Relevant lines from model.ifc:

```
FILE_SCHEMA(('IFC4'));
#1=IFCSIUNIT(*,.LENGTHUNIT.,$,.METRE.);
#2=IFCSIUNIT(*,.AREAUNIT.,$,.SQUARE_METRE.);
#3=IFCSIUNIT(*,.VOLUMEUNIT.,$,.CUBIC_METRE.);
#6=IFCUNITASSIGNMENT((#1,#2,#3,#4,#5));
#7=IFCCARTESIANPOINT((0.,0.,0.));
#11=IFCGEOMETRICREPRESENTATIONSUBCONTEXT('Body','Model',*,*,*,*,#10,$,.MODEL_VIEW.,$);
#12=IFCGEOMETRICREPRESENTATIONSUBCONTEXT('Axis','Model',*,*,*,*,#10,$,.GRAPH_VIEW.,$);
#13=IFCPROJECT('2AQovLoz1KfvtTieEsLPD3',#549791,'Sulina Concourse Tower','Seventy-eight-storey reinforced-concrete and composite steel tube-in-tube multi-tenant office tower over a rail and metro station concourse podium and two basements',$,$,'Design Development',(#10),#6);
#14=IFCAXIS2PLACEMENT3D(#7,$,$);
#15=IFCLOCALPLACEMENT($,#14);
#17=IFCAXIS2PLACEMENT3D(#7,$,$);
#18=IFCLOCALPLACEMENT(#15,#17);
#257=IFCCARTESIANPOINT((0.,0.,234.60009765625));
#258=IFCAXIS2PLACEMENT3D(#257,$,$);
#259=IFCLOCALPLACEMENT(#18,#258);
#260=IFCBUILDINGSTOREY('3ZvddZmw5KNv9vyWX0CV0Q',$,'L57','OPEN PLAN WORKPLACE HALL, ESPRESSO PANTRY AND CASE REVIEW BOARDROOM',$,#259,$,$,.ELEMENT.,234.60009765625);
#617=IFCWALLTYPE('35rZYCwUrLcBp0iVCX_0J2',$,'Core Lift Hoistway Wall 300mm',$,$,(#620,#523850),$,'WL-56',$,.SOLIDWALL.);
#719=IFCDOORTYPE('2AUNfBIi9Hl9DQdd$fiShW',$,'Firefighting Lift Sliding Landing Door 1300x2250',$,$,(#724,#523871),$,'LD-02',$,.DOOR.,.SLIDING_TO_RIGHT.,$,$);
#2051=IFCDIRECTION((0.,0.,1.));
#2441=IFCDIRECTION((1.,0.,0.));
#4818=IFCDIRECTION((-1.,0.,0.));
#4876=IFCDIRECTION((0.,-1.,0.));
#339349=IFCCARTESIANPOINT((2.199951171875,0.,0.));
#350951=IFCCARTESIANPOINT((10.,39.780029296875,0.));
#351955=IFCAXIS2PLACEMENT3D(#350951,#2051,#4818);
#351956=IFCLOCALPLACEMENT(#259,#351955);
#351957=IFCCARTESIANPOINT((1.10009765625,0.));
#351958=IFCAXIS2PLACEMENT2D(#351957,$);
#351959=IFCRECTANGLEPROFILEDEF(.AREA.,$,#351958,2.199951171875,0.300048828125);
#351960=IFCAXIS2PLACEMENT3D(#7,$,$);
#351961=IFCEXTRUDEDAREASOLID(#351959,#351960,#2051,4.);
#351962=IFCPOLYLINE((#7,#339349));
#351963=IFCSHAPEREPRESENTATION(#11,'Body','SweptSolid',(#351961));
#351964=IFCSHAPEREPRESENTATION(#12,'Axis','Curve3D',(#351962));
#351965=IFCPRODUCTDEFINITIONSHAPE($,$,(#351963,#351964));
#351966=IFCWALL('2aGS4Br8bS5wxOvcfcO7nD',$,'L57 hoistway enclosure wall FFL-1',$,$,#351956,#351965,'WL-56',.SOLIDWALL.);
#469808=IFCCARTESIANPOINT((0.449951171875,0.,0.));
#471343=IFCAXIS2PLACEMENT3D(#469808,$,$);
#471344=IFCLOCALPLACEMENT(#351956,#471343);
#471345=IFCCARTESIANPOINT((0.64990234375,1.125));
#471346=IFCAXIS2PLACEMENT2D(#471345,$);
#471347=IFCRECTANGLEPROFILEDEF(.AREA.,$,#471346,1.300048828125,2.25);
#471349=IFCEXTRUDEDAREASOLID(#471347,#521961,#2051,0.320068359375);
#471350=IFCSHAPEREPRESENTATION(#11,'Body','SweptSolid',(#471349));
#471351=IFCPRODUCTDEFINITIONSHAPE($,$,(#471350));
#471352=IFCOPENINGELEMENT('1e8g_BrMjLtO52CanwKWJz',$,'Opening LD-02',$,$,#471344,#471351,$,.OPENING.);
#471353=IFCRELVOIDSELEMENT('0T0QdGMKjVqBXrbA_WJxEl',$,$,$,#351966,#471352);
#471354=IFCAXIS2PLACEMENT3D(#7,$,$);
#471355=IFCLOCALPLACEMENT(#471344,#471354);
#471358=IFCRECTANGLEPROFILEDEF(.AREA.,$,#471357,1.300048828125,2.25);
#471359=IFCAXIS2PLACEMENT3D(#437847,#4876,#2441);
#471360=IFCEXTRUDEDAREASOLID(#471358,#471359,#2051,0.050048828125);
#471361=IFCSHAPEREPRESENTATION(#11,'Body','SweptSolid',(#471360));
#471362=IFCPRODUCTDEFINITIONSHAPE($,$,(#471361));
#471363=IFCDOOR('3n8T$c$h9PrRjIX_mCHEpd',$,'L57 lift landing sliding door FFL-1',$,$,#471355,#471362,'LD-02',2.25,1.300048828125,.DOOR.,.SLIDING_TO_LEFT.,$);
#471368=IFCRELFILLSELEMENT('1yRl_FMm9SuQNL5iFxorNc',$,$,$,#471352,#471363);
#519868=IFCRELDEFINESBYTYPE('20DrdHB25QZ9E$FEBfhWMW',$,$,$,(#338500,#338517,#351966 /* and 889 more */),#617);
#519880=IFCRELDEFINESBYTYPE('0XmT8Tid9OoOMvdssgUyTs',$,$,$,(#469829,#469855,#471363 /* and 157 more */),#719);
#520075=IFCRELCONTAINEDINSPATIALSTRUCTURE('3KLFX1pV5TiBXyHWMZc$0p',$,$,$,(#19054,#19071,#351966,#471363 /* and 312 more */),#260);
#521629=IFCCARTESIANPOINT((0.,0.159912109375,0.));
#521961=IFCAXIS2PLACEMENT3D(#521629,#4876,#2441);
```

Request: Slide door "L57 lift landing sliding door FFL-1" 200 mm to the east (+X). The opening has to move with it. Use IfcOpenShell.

```python
import ifcopenshell
import ifcopenshell.api.geometry
import ifcopenshell.util.placement
import ifcopenshell.util.unit

model = ifcopenshell.open("model.ifc")
unit_scale = ifcopenshell.util.unit.calculate_unit_scale(model)

door = model.by_guid("3n8T$c$h9PrRjIX_mCHEpd")
opening = door.FillsVoids[0].RelatingOpeningElement
wall = opening.VoidsElements[0].RelatingBuildingElement

wall_matrix = ifcopenshell.util.placement.get_local_placement(wall.ObjectPlacement)
shift = wall_matrix[:3, 0] * -0.2 / unit_scale
before = ifcopenshell.util.placement.get_local_placement(door.ObjectPlacement)[:3, 3].copy()

# The door is placed relative to its opening, so it follows when the opening moves.
matrix = ifcopenshell.util.placement.get_local_placement(opening.ObjectPlacement)
matrix[:3, 3] += shift
ifcopenshell.api.geometry.edit_object_placement(
    model, product=opening, matrix=matrix, is_si=False, should_transform_children=True
)

after = ifcopenshell.util.placement.get_local_placement(door.ObjectPlacement)[:3, 3]
print("door moved by", (after - before).round(3) + 0.0)

model.write("model_v2.ifc")
```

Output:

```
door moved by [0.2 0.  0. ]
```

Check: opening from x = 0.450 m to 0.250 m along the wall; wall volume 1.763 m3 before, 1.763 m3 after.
